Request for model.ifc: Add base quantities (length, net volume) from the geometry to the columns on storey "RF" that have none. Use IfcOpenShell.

First a look at what the model holds.

```python
import ifcopenshell
import ifcopenshell.util.element
import ifcopenshell.util.unit

model = ifcopenshell.open("model.ifc")
print(model.schema)
for unit_type in ("LENGTHUNIT", "AREAUNIT", "VOLUMEUNIT"):
    print(unit_type, ifcopenshell.util.unit.calculate_unit_scale(model, unit_type))
storey = next(s for s in model.by_type("IfcBuildingStorey") if s.Name == "RF")
columns = [e for e in ifcopenshell.util.element.get_decomposition(storey) if e.is_a("IfcColumn")]
for e in sorted(columns, key=lambda e: e.id()):
    print(e.id(), e.is_a(), e.Name, list(ifcopenshell.util.element.get_psets(e, qtos_only=True)), sep=" | ")
```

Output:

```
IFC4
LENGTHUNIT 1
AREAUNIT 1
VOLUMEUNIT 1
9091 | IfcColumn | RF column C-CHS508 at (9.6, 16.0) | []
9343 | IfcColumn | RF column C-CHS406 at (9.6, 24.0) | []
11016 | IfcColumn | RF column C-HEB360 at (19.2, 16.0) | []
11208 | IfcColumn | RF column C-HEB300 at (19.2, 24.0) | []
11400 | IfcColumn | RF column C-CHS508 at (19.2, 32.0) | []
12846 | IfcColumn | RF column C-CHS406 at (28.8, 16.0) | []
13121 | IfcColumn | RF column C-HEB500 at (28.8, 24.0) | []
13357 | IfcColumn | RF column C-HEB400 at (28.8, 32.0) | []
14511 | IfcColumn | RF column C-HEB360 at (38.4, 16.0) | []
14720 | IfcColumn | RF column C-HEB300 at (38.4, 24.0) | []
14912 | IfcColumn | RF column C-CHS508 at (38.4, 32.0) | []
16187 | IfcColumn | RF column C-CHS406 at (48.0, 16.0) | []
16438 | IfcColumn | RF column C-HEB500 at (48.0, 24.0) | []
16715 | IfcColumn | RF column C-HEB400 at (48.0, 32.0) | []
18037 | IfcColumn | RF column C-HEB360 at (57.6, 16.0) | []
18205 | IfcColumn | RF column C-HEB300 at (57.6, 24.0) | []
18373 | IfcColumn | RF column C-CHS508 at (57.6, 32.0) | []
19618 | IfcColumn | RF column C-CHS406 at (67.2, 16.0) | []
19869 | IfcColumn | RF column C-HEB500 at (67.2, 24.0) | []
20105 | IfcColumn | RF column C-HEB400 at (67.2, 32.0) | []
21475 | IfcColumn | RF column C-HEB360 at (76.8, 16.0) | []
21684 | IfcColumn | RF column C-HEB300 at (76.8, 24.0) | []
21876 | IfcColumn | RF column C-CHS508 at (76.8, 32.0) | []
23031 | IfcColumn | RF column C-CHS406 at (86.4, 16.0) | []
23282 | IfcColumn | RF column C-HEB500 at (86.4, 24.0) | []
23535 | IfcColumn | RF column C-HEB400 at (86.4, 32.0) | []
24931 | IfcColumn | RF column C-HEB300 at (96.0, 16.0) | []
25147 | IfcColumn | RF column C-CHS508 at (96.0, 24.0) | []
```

```python
import ifcopenshell
import ifcopenshell.api.pset
import ifcopenshell.geom
import ifcopenshell.util.element
import ifcopenshell.util.shape
import ifcopenshell.util.unit

model = ifcopenshell.open("model.ifc")
unit_scale = ifcopenshell.util.unit.calculate_unit_scale(model)
volume_scale = ifcopenshell.util.unit.calculate_unit_scale(model, "VOLUMEUNIT")
settings = ifcopenshell.geom.settings()

storey = next(s for s in model.by_type("IfcBuildingStorey") if s.Name == "RF")
columns = [e for e in ifcopenshell.util.element.get_decomposition(storey) if e.is_a("IfcColumn")]

for e in sorted(columns, key=lambda e: e.id()):
    if ifcopenshell.util.element.get_psets(e, qtos_only=True, should_inherit=False):
        continue
    # Geometry comes back in metres, in the element's own axes.
    shape = ifcopenshell.geom.create_shape(settings, e)
    values = {
        "Length": ifcopenshell.util.shape.get_z(shape.geometry) / unit_scale,
        "NetVolume": ifcopenshell.util.shape.get_volume(shape.geometry) / volume_scale,
    }
    qto = ifcopenshell.api.pset.add_qto(model, product=e, name="Qto_ColumnBaseQuantities")
    ifcopenshell.api.pset.edit_qto(model, qto=qto, properties=values)
    print(e.id(), {k: round(v, 3) for k, v in values.items()})

model.write("model-out.ifc")
```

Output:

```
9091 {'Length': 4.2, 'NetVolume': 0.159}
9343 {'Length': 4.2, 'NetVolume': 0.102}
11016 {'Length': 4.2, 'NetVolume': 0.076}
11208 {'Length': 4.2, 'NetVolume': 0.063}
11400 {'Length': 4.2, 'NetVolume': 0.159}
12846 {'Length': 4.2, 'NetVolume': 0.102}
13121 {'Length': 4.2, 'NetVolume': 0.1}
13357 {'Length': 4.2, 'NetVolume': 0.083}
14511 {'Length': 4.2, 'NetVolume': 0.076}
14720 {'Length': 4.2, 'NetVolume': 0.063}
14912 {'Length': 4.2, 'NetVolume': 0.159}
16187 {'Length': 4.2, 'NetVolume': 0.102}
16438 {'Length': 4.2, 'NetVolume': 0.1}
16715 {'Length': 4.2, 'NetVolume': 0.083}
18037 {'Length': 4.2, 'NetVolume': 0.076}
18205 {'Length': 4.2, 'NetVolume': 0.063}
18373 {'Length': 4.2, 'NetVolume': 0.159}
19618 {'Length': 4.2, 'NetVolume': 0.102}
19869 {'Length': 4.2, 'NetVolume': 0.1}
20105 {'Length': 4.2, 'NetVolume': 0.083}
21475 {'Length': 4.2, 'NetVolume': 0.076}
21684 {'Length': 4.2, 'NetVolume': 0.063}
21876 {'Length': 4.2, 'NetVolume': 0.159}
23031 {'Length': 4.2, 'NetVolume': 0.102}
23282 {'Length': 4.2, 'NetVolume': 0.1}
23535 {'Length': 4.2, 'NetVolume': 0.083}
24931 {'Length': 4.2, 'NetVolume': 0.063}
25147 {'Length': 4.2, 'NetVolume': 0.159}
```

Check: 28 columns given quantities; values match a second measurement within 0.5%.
